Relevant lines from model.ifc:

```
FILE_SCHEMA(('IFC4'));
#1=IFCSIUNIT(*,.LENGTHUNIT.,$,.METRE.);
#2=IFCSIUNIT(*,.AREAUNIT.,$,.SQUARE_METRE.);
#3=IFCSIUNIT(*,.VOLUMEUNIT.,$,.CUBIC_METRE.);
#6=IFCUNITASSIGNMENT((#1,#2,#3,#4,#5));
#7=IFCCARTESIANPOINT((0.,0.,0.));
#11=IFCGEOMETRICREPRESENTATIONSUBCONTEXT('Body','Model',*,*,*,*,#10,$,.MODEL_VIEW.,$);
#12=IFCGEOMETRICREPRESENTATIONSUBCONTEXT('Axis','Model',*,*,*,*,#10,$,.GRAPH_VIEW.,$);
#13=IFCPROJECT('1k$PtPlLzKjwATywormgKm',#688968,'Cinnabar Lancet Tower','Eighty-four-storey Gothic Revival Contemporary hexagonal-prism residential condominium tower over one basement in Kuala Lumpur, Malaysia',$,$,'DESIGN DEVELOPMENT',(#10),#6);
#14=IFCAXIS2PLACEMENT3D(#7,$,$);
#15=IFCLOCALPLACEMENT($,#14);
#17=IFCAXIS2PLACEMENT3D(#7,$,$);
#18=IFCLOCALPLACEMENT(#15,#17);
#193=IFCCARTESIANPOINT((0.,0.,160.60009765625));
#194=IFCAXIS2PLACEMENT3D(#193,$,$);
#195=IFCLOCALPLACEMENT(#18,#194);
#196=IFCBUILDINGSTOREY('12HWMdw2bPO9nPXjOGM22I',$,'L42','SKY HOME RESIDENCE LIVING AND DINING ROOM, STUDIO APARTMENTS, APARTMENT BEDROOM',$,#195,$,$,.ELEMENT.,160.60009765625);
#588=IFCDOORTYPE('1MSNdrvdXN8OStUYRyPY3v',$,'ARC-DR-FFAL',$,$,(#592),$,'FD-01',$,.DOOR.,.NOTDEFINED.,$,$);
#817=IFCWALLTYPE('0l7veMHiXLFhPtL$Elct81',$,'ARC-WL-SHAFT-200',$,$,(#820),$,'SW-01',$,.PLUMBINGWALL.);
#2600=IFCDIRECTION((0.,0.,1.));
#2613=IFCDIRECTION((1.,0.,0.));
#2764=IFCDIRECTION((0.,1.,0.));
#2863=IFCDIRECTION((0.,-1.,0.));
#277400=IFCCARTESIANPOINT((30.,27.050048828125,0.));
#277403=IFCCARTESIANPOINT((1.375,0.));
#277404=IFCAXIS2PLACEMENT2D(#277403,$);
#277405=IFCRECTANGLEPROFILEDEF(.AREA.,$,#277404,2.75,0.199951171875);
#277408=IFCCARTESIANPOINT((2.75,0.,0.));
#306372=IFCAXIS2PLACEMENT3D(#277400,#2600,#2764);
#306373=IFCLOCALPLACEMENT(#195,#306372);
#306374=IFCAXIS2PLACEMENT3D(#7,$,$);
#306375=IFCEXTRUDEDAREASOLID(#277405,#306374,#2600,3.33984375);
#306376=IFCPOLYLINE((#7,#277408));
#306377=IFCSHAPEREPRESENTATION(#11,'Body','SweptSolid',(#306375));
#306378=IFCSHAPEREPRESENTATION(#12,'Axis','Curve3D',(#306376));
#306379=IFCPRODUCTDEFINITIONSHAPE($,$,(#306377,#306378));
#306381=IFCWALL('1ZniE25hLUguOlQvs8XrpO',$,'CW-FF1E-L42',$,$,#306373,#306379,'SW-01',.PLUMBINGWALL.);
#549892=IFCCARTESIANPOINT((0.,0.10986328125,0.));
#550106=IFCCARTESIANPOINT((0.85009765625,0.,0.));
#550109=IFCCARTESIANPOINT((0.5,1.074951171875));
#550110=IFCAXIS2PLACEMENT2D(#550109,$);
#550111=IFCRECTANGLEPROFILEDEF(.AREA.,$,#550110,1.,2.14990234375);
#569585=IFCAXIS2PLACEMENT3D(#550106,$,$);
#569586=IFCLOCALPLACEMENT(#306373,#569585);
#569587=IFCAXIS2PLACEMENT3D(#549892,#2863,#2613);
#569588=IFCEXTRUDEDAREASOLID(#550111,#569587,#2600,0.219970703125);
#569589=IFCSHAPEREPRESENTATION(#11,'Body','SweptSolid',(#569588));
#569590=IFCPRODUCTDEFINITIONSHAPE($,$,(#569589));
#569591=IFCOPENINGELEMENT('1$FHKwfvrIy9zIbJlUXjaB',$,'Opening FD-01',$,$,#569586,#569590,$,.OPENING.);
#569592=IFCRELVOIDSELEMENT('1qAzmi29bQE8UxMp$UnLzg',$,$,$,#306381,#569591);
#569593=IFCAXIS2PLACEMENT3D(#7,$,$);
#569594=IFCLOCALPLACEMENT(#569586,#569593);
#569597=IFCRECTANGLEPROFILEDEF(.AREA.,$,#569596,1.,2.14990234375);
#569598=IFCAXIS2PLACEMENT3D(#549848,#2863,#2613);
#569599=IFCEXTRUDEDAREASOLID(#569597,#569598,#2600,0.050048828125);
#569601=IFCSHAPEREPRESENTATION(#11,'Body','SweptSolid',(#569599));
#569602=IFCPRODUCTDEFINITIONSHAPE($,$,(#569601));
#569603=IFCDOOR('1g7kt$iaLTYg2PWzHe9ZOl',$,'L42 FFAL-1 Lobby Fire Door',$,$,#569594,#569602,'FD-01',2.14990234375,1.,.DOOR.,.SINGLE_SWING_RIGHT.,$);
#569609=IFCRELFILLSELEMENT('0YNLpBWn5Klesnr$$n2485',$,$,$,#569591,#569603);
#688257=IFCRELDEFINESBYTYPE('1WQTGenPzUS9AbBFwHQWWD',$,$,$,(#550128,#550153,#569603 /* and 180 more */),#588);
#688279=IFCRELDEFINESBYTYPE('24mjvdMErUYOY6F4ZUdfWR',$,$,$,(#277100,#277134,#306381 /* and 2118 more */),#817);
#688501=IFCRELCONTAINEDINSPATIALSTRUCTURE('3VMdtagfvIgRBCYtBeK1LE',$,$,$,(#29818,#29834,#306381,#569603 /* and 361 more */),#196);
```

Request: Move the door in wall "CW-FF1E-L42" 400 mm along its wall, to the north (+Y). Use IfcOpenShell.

```python
import ifcopenshell
import ifcopenshell.api.geometry
import ifcopenshell.util.placement

model = ifcopenshell.open("model.ifc")

door = model.by_guid("1g7kt$iaLTYg2PWzHe9ZOl")
opening = door.FillsVoids[0].RelatingOpeningElement
wall = opening.VoidsElements[0].RelatingBuildingElement

wall_matrix = ifcopenshell.util.placement.get_local_placement(wall.ObjectPlacement)
shift = wall_matrix[:3, 0] * 0.4
before = ifcopenshell.util.placement.get_local_placement(door.ObjectPlacement)[:3, 3].copy()

# The door is placed relative to its opening, so it follows when the opening moves.
matrix = ifcopenshell.util.placement.get_local_placement(opening.ObjectPlacement)
matrix[:3, 3] += shift
ifcopenshell.api.geometry.edit_object_placement(
    model, product=opening, matrix=matrix, is_si=False, should_transform_children=True
)

after = ifcopenshell.util.placement.get_local_placement(door.ObjectPlacement)[:3, 3]
print("door moved by", (after - before).round(3) + 0.0)

model.write("model_v2.ifc")
```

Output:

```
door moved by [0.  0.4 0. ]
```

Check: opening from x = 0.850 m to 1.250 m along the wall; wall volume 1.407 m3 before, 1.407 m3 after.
